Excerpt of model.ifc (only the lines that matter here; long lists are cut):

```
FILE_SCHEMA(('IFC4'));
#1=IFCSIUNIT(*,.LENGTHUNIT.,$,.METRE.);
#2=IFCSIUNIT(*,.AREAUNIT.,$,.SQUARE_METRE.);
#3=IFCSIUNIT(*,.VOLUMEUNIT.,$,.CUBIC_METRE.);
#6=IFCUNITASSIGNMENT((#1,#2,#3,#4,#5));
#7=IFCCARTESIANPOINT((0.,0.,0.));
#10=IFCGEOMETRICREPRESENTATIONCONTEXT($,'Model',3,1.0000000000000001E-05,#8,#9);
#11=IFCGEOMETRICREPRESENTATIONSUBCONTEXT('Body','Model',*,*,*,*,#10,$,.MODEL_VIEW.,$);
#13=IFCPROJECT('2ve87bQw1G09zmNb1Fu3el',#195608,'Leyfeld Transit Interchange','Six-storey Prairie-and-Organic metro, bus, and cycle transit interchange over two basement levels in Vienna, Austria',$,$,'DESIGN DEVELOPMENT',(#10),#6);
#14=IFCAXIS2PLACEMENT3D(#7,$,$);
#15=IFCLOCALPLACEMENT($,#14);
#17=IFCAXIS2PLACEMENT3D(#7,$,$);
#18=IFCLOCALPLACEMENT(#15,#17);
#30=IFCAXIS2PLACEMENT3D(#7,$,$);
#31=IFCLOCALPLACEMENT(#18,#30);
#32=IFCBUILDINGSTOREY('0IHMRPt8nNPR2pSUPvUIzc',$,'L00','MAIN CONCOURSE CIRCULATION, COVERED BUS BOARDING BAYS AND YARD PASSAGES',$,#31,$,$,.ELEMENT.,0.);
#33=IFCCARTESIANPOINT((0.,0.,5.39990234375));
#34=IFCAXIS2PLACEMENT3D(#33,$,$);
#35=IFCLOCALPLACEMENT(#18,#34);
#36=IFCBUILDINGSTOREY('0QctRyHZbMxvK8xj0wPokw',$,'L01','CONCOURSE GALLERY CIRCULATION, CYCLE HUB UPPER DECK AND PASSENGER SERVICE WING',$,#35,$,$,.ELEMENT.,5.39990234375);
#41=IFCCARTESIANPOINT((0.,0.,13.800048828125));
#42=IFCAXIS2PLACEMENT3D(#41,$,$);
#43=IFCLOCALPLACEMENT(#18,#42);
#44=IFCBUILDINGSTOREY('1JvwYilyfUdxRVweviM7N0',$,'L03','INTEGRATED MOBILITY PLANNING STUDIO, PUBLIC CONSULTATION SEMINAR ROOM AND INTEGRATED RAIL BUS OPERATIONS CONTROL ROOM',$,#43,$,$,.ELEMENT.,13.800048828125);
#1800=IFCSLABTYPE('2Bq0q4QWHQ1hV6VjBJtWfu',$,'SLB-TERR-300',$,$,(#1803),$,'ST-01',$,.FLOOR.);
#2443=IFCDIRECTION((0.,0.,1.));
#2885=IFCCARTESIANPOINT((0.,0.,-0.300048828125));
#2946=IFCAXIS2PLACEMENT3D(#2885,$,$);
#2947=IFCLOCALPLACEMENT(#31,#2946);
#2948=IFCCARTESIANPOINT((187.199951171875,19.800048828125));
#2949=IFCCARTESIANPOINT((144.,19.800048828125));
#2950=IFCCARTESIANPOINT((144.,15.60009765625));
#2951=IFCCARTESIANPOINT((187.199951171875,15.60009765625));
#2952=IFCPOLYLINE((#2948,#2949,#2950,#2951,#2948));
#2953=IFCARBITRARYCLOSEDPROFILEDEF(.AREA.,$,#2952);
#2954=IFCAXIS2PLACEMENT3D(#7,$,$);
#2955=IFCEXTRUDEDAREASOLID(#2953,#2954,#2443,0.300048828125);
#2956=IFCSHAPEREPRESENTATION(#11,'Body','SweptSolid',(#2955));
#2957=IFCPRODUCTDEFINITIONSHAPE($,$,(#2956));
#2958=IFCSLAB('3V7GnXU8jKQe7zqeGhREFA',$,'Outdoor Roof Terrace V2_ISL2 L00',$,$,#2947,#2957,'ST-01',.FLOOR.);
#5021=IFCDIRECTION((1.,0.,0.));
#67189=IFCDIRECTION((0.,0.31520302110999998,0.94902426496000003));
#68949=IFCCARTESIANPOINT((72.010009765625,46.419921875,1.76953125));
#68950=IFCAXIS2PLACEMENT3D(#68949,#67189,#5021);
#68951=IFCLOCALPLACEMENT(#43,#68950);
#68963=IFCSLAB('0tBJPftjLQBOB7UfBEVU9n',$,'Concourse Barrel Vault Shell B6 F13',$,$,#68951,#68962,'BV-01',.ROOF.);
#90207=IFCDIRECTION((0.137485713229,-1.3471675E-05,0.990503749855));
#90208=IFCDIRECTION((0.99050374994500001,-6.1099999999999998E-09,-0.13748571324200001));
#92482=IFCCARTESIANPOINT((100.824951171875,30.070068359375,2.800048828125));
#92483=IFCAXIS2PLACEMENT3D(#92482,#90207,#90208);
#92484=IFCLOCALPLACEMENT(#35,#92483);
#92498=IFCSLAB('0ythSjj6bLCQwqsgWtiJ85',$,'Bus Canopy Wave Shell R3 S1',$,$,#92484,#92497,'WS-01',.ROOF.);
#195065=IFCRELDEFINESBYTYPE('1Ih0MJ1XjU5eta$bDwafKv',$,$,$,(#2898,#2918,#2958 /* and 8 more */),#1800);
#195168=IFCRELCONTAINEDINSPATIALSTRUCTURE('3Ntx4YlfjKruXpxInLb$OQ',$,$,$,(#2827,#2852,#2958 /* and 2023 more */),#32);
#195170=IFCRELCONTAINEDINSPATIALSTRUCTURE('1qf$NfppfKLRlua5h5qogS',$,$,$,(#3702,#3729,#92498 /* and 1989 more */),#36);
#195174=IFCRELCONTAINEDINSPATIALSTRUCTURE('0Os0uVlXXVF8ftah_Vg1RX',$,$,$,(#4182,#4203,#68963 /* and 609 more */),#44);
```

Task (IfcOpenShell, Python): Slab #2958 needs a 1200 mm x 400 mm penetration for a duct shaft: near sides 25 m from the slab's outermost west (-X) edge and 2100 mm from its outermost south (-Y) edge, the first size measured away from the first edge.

```python
import numpy as np
import ifcopenshell
import ifcopenshell.api.feature
import ifcopenshell.api.geometry
import ifcopenshell.api.root
import ifcopenshell.geom
import ifcopenshell.util.placement
import ifcopenshell.util.representation
import ifcopenshell.util.shape
import ifcopenshell.util.unit

model = ifcopenshell.open("model.ifc")
unit_scale = ifcopenshell.util.unit.calculate_unit_scale(model)
settings = ifcopenshell.geom.settings()


def volume(element):
    """Net volume in cubic metres, openings subtracted."""
    shape = ifcopenshell.geom.create_shape(settings, element)
    return ifcopenshell.util.shape.get_volume(shape.geometry)


slab = model.by_guid("3V7GnXU8jKQe7zqeGhREFA")
before = volume(slab)

# Extent in the slab's own axes, in metres. The edges named are its -X and -Y sides.
slab_shape = ifcopenshell.geom.create_shape(settings, slab)
vertices = ifcopenshell.util.shape.get_vertices(slab_shape.geometry)
x_min, y_min, bottom = vertices.min(axis=0)
top = vertices[:, 2].max()

opening = ifcopenshell.api.root.create_entity(model, ifc_class="IfcOpeningElement", name="Duct shaft opening", predefined_type="OPENING")
context = ifcopenshell.util.representation.get_context(model, "Model", "Body", "MODEL_VIEW")
width, depth = 1.2, 0.4
outline = [(0.0, 0.0), (width, 0.0), (width, depth), (0.0, depth), (0.0, 0.0)]
# Overshoot both faces by 50 mm so the cut is clean.
shape = ifcopenshell.api.geometry.add_slab_representation(
    model, context=context, depth=top - bottom + 0.1, polyline=outline
)
ifcopenshell.api.geometry.assign_representation(model, product=opening, representation=shape)

matrix = ifcopenshell.util.placement.get_local_placement(slab.ObjectPlacement)
matrix[:, 3] = matrix @ np.append(np.array([x_min + 25, y_min + 2.1, bottom - 0.05]) / unit_scale, 1.0)
ifcopenshell.api.geometry.edit_object_placement(model, product=opening, matrix=matrix, is_si=False)
ifcopenshell.api.feature.add_feature(model, feature=opening, element=slab)

after = volume(slab)

print(f"slab volume {before:.3f} -> {after:.3f} m3")

model.write("model_updated.ifc")
```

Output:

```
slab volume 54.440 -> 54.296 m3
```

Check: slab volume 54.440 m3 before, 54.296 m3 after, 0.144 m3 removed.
